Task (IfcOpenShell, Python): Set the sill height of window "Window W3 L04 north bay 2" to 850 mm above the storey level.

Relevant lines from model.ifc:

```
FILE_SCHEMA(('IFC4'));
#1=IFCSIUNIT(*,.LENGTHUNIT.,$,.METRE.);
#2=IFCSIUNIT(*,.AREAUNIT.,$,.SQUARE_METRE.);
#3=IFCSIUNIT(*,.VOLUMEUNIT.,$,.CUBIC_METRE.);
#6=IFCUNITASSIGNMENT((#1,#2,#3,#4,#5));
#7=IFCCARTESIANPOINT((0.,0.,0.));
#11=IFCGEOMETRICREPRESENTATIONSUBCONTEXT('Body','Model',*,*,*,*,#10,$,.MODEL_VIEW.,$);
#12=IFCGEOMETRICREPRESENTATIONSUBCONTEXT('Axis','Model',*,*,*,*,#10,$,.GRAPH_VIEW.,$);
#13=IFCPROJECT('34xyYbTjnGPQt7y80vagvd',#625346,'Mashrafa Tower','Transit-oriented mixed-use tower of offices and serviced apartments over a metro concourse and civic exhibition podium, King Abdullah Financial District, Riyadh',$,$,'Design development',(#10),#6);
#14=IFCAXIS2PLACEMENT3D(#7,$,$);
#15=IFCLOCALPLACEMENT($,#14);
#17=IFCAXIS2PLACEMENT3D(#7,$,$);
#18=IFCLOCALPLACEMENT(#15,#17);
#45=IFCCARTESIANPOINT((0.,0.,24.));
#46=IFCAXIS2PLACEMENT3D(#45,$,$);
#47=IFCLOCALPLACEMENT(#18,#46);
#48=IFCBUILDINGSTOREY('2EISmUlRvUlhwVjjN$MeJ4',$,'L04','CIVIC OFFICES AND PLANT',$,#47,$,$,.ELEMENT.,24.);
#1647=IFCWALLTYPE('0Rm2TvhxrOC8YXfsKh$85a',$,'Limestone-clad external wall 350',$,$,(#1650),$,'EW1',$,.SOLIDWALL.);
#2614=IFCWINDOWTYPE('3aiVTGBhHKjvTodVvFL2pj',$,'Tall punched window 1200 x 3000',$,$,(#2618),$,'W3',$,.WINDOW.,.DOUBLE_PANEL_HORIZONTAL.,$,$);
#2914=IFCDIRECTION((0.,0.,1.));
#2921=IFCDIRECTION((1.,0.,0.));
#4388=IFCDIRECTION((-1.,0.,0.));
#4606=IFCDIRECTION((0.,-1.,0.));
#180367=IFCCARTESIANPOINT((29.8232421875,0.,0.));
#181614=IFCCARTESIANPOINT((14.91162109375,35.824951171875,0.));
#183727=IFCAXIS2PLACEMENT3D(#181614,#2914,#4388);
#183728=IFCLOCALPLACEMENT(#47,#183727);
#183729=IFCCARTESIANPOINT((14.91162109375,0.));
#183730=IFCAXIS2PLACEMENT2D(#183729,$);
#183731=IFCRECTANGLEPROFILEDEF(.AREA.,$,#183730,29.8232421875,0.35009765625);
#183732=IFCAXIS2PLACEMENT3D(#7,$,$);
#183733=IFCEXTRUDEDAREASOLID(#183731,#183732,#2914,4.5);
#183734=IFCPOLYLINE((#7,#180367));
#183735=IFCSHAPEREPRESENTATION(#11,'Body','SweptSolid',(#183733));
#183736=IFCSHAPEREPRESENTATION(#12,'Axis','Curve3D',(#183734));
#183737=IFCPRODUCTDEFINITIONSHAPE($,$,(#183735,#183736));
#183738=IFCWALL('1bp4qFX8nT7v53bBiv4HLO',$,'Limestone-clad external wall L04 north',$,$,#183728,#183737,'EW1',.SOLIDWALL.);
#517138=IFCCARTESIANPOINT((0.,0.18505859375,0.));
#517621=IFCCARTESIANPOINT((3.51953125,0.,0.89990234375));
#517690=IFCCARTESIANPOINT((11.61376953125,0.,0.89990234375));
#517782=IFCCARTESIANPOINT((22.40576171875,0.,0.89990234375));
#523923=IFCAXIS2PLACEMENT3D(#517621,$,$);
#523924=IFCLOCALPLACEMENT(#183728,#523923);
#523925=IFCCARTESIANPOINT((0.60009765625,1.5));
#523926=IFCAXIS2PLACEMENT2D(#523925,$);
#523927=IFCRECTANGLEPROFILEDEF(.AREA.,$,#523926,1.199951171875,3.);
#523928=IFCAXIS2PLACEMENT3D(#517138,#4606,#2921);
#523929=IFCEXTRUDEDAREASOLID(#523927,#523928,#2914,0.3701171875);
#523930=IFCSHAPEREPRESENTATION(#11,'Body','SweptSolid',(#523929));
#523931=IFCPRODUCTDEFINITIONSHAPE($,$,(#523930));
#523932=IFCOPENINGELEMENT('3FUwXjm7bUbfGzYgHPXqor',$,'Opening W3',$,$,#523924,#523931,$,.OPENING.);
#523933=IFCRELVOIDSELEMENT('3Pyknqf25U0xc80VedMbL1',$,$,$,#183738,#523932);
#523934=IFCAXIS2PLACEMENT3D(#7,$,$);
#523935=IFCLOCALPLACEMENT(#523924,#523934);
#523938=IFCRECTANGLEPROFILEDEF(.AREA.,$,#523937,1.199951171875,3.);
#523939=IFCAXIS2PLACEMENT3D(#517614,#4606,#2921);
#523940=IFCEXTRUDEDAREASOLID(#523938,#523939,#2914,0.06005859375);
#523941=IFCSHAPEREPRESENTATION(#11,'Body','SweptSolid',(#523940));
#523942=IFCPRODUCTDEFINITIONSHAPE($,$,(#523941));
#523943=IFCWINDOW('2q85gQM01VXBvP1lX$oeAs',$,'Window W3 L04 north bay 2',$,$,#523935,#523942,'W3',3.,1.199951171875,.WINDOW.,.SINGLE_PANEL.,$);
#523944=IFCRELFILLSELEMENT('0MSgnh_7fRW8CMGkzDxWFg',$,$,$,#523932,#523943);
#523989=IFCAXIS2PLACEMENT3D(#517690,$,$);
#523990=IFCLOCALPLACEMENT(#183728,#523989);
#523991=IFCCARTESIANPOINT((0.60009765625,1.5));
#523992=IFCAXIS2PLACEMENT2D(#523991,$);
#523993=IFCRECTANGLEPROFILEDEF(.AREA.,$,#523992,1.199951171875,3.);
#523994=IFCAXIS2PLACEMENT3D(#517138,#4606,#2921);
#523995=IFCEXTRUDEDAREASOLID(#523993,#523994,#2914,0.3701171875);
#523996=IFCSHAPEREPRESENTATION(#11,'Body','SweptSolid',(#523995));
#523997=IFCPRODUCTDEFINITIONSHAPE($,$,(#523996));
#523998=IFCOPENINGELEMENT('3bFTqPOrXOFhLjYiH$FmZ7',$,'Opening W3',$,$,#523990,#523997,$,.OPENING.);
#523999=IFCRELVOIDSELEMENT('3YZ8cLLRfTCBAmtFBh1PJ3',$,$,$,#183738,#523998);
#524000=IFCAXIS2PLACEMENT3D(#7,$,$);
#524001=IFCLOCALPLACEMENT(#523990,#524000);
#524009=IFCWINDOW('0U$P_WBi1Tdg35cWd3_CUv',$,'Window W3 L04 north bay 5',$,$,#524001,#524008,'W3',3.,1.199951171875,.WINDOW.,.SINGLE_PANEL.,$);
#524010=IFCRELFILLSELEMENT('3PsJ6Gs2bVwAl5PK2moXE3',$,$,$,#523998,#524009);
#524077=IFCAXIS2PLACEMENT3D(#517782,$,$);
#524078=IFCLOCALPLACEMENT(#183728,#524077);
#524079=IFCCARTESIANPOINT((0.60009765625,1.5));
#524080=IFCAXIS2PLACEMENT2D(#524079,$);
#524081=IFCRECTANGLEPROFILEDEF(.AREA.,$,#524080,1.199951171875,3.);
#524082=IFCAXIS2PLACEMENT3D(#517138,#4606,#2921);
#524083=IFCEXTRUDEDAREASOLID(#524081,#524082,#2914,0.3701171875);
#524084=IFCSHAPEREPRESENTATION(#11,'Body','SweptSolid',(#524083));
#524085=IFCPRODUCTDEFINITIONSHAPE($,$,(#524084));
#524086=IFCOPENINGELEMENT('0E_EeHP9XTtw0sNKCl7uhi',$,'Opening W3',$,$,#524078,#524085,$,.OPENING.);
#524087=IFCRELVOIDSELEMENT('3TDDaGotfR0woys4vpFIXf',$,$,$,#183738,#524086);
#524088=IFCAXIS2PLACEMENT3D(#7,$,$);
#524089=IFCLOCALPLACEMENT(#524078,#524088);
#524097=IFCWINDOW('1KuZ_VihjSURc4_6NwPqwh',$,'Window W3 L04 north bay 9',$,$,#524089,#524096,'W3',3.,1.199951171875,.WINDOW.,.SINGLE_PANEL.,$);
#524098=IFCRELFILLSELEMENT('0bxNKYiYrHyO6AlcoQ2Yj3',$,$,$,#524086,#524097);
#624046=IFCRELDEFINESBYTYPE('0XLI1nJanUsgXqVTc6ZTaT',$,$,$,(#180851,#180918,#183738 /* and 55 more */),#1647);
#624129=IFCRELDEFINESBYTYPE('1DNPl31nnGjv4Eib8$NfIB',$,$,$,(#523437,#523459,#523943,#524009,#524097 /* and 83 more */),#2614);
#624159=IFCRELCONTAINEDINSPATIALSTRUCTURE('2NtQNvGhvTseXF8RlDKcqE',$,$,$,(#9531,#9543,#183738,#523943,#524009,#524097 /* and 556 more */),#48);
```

```python
import numpy as np
import ifcopenshell
import ifcopenshell.api.geometry
import ifcopenshell.geom
import ifcopenshell.util.element
import ifcopenshell.util.placement
import ifcopenshell.util.shape
import ifcopenshell.util.unit

model = ifcopenshell.open("model.ifc")
unit_scale = ifcopenshell.util.unit.calculate_unit_scale(model)

window = model.by_guid("2q85gQM01VXBvP1lX$oeAs")
opening = window.FillsVoids[0].RelatingOpeningElement
storey = ifcopenshell.util.element.get_container(window, ifc_class="IfcBuildingStorey")
level = ifcopenshell.util.placement.get_local_placement(storey.ObjectPlacement)[2, 3]

# The opening's origin need not be at the sill, so measure its lowest point.
shape = ifcopenshell.geom.create_shape(ifcopenshell.geom.settings(), opening)
bottom = ifcopenshell.util.shape.get_shape_bottom_elevation(shape, shape.geometry) / unit_scale
dz = level + 0.85 / unit_scale - bottom

shift = np.array([0.0, 0.0, dz])
# The window is placed relative to its opening, so it follows when the opening moves.
matrix = ifcopenshell.util.placement.get_local_placement(opening.ObjectPlacement)
matrix[:3, 3] += shift
ifcopenshell.api.geometry.edit_object_placement(
    model, product=opening, matrix=matrix, is_si=False, should_transform_children=True
)

print(f"moved by {dz * unit_scale:+.3f} m")

model.write("model_edited.ifc")
```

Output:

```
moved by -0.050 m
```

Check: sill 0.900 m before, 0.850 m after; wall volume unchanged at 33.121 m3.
